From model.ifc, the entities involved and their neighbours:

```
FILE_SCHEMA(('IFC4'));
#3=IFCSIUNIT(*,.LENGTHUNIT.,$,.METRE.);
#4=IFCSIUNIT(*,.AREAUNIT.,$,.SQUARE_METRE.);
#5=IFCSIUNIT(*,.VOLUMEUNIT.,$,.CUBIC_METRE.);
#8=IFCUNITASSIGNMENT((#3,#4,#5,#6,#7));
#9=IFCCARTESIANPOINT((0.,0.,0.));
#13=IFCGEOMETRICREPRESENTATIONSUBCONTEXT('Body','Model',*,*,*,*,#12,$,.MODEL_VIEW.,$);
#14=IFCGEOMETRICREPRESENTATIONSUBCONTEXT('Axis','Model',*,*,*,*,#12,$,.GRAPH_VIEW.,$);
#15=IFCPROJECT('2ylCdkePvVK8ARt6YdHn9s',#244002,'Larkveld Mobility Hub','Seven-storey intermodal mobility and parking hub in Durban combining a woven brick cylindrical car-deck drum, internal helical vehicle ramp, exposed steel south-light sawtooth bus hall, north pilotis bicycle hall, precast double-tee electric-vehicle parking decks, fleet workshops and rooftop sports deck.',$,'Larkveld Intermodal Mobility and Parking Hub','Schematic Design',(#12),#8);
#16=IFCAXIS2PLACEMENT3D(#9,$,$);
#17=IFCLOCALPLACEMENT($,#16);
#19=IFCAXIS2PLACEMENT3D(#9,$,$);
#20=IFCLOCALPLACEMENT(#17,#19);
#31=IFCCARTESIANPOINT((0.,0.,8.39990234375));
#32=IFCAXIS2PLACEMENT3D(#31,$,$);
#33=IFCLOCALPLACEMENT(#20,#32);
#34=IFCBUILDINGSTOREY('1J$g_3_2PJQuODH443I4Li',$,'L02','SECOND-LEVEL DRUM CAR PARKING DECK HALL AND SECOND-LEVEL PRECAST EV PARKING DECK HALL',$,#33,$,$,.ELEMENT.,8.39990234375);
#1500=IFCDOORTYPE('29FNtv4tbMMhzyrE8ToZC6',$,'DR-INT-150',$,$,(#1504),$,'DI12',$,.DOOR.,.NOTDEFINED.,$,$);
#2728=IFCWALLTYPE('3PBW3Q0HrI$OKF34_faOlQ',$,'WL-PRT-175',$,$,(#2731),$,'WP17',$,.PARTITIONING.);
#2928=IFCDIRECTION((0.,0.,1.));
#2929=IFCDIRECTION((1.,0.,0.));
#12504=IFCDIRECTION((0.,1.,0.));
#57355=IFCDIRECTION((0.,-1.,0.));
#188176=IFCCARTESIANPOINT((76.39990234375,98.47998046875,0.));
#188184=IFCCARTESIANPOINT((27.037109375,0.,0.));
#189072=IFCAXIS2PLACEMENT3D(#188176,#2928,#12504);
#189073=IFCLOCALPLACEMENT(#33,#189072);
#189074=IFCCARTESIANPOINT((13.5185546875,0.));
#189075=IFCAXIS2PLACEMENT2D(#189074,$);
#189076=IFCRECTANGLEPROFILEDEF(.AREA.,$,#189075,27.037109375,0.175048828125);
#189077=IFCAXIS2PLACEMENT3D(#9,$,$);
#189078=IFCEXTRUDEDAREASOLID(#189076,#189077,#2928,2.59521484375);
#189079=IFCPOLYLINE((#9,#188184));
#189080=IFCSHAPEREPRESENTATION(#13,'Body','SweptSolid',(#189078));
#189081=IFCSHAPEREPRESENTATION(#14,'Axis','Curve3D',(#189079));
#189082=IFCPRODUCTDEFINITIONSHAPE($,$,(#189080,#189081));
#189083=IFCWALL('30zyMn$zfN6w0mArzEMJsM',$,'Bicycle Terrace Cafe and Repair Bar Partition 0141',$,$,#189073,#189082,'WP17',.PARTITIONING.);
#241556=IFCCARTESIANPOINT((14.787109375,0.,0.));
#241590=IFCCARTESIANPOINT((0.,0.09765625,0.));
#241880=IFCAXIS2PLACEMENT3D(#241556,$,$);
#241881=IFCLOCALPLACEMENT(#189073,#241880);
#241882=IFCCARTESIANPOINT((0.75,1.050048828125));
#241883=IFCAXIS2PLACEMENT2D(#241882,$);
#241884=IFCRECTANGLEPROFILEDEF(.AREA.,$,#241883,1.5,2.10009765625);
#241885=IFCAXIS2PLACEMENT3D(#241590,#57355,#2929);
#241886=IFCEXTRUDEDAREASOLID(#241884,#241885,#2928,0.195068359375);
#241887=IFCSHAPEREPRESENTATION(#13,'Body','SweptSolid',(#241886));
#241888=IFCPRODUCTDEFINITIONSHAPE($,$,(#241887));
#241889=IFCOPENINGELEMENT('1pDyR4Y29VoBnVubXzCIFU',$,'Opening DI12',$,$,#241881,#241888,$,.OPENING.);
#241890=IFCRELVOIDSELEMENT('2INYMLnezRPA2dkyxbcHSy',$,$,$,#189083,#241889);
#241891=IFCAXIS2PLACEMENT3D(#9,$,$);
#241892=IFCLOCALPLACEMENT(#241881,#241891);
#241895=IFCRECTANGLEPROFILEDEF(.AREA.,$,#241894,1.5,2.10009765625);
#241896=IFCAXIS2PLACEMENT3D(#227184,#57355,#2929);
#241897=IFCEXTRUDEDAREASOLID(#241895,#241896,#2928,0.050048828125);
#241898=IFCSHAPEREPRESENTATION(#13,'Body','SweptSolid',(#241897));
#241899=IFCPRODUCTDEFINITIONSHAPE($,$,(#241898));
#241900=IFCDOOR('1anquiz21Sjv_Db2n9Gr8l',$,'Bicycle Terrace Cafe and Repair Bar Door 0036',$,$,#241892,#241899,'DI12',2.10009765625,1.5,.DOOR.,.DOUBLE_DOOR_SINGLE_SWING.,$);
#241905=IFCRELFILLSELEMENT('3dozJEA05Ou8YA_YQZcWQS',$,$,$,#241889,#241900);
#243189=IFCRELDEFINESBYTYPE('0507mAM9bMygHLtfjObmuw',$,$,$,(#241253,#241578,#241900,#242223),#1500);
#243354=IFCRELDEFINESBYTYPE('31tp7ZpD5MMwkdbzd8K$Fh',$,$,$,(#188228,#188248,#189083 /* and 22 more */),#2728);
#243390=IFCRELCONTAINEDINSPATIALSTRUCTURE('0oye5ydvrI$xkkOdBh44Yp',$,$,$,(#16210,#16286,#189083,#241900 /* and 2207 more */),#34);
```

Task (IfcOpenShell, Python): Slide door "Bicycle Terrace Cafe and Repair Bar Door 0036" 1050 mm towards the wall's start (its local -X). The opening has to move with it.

```python
import ifcopenshell
import ifcopenshell.api.geometry
import ifcopenshell.util.placement

model = ifcopenshell.open("model.ifc")

door = model.by_id(241900)
opening = door.FillsVoids[0].RelatingOpeningElement
wall = opening.VoidsElements[0].RelatingBuildingElement

wall_matrix = ifcopenshell.util.placement.get_local_placement(wall.ObjectPlacement)
shift = wall_matrix[:3, 0] * -1.05
before = ifcopenshell.util.placement.get_local_placement(door.ObjectPlacement)[:3, 3].copy()

# The door is placed relative to its opening, so it follows when the opening moves.
matrix = ifcopenshell.util.placement.get_local_placement(opening.ObjectPlacement)
matrix[:3, 3] += shift
ifcopenshell.api.geometry.edit_object_placement(
    model, product=opening, matrix=matrix, is_si=False, should_transform_children=True
)

after = ifcopenshell.util.placement.get_local_placement(door.ObjectPlacement)[:3, 3]
print("door moved by", (after - before).round(3) + 0.0)

model.write("model_updated.ifc")
```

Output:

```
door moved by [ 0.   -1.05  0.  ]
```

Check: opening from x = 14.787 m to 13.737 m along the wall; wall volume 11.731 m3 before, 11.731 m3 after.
